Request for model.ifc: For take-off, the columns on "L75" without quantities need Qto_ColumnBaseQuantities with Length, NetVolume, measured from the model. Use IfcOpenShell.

First a look at what the model holds.

```python
import ifcopenshell
import ifcopenshell.util.element
import ifcopenshell.util.unit

model = ifcopenshell.open("model.ifc")
print(model.schema)
for unit_type in ("LENGTHUNIT", "AREAUNIT", "VOLUMEUNIT"):
    print(unit_type, ifcopenshell.util.unit.calculate_unit_scale(model, unit_type))
storey = next(s for s in model.by_type("IfcBuildingStorey") if s.Name == "L75")
columns = [e for e in ifcopenshell.util.element.get_decomposition(storey) if e.is_a("IfcColumn")]
for e in sorted(columns, key=lambda e: e.id()):
    print(e.id(), e.is_a(), e.Name, list(ifcopenshell.util.element.get_psets(e, qtos_only=True)), sep=" | ")
```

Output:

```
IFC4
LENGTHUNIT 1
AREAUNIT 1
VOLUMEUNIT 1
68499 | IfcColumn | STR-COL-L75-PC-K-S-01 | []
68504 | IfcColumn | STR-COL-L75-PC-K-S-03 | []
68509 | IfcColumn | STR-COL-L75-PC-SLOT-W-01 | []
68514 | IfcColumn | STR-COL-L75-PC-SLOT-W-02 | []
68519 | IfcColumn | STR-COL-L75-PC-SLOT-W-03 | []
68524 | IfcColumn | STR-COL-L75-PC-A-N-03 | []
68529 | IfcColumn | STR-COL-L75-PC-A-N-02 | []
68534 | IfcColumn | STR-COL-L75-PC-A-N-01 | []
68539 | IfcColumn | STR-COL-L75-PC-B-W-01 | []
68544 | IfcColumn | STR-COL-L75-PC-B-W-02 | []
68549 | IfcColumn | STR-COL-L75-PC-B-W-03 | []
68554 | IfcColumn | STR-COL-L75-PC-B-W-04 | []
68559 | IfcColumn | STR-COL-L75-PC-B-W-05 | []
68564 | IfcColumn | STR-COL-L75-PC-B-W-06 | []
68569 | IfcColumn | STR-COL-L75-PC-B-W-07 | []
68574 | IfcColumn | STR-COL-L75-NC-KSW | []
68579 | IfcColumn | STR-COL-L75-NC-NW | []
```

```python
import ifcopenshell
import ifcopenshell.api.pset
import ifcopenshell.geom
import ifcopenshell.util.element
import ifcopenshell.util.shape
import ifcopenshell.util.unit

model = ifcopenshell.open("model.ifc")
unit_scale = ifcopenshell.util.unit.calculate_unit_scale(model)
volume_scale = ifcopenshell.util.unit.calculate_unit_scale(model, "VOLUMEUNIT")
settings = ifcopenshell.geom.settings()

storey = next(s for s in model.by_type("IfcBuildingStorey") if s.Name == "L75")
columns = [e for e in ifcopenshell.util.element.get_decomposition(storey) if e.is_a("IfcColumn")]

for e in sorted(columns, key=lambda e: e.id()):
    if ifcopenshell.util.element.get_psets(e, qtos_only=True, should_inherit=False):
        continue
    # Geometry comes back in metres, in the element's own axes.
    shape = ifcopenshell.geom.create_shape(settings, e)
    values = {
        "Length": ifcopenshell.util.shape.get_z(shape.geometry) / unit_scale,
        "NetVolume": ifcopenshell.util.shape.get_volume(shape.geometry) / volume_scale,
    }
    qto = ifcopenshell.api.pset.add_qto(model, product=e, name="Qto_ColumnBaseQuantities")
    ifcopenshell.api.pset.edit_qto(model, qto=qto, properties=values)
    print(e.id(), {k: round(v, 3) for k, v in values.items()})

model.write("model_updated.ifc")
```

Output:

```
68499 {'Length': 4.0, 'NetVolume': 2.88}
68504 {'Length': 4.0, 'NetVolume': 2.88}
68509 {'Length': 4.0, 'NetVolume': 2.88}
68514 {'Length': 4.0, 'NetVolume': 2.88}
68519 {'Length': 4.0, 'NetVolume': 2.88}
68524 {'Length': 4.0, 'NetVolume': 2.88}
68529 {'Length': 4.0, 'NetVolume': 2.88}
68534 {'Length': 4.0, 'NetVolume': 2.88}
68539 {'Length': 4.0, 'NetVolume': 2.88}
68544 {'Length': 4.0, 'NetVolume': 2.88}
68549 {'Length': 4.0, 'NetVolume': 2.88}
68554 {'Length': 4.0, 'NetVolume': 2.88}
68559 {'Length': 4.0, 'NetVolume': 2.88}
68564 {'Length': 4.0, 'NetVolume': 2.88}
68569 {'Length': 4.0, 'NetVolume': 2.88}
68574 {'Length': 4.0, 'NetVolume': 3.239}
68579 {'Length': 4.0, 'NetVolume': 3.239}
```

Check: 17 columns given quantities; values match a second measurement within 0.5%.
